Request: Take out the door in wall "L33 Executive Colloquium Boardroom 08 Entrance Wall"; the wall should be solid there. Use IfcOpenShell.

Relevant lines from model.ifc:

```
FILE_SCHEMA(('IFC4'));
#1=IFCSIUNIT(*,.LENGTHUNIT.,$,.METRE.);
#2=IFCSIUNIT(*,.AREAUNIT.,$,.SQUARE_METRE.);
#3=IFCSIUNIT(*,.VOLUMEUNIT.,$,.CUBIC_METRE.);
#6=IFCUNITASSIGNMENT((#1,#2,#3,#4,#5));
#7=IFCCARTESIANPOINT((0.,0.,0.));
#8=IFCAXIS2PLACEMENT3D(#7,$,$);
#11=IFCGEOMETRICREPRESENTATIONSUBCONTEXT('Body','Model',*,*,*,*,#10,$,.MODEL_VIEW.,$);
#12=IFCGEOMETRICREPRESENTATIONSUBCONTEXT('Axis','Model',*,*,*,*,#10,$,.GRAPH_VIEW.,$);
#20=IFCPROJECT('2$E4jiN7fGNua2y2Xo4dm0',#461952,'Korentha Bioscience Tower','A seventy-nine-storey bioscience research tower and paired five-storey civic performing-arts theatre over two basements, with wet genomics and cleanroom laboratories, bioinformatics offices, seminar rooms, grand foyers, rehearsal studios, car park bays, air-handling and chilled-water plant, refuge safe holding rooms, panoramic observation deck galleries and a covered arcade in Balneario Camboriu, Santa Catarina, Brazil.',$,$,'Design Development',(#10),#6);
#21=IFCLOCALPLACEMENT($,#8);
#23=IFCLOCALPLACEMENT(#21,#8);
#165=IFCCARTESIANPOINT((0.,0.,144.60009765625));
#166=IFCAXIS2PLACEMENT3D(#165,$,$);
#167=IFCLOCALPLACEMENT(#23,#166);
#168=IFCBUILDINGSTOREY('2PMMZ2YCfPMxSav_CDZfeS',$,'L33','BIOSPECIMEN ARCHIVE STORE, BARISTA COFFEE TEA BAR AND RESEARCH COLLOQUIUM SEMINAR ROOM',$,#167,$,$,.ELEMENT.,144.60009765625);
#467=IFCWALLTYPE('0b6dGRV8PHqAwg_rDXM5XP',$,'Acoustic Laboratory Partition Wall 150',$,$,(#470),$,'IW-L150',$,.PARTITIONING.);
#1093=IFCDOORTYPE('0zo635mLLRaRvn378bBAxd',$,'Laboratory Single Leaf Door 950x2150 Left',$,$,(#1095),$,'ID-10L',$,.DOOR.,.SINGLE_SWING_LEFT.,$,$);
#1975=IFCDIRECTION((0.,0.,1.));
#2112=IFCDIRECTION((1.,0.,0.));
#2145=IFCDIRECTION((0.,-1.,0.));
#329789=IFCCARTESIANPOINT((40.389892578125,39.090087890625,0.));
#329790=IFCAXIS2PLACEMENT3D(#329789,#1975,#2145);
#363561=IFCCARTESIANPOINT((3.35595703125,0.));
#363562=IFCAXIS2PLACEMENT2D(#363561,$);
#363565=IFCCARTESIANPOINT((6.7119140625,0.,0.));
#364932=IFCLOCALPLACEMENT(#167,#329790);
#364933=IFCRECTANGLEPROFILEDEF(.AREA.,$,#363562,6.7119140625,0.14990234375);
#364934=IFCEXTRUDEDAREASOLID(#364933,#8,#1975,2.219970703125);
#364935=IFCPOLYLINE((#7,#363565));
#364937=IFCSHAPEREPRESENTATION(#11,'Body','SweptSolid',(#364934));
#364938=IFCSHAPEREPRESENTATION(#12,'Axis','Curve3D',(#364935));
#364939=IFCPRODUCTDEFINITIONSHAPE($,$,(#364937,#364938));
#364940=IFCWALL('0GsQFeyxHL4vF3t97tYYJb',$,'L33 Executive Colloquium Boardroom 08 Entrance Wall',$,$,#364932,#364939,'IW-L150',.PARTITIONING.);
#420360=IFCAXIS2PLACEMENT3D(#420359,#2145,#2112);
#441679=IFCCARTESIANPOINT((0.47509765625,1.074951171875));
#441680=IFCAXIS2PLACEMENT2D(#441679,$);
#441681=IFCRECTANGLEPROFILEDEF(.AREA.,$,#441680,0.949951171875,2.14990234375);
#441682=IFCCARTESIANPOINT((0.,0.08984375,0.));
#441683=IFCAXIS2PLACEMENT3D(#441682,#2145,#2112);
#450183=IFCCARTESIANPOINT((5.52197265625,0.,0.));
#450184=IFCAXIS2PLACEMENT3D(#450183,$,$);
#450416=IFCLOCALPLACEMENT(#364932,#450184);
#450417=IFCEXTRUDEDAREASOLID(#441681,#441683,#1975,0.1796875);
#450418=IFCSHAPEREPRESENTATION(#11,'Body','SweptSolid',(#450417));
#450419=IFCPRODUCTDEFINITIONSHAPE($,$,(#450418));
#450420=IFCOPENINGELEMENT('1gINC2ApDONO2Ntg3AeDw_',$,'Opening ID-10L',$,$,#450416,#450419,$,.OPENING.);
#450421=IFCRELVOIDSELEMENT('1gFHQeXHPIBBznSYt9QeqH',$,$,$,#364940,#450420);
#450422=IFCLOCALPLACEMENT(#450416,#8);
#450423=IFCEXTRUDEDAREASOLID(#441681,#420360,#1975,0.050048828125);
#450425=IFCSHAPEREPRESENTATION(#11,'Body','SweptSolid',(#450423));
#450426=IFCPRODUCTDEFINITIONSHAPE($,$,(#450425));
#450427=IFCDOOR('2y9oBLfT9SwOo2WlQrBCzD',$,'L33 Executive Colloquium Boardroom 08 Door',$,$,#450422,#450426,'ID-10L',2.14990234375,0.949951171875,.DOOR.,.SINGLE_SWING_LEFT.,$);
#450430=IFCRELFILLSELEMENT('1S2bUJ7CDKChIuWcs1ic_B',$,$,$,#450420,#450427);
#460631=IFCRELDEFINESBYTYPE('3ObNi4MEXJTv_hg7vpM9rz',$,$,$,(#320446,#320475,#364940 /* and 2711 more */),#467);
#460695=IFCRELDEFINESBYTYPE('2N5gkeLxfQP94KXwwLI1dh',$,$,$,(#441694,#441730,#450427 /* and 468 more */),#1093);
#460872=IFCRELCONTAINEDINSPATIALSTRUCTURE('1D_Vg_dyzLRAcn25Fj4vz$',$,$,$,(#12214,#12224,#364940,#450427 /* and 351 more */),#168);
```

```python
import ifcopenshell
import ifcopenshell.api.feature
import ifcopenshell.api.root
import ifcopenshell.geom
import ifcopenshell.util.shape

model = ifcopenshell.open("model.ifc")
settings = ifcopenshell.geom.settings()


def volume(element):
    """Net volume in cubic metres, openings subtracted."""
    shape = ifcopenshell.geom.create_shape(settings, element)
    return ifcopenshell.util.shape.get_volume(shape.geometry)


door = model.by_id(450427)
opening = door.FillsVoids[0].RelatingOpeningElement
wall = opening.VoidsElements[0].RelatingBuildingElement
before = volume(wall)

ifcopenshell.api.root.remove_product(model, product=door)
ifcopenshell.api.feature.remove_feature(model, feature=opening)

after = volume(wall)

print(f"wall volume {before:.3f} -> {after:.3f} m3")

model.write("model_updated.ifc")
```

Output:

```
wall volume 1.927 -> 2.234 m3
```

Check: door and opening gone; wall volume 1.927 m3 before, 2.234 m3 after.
